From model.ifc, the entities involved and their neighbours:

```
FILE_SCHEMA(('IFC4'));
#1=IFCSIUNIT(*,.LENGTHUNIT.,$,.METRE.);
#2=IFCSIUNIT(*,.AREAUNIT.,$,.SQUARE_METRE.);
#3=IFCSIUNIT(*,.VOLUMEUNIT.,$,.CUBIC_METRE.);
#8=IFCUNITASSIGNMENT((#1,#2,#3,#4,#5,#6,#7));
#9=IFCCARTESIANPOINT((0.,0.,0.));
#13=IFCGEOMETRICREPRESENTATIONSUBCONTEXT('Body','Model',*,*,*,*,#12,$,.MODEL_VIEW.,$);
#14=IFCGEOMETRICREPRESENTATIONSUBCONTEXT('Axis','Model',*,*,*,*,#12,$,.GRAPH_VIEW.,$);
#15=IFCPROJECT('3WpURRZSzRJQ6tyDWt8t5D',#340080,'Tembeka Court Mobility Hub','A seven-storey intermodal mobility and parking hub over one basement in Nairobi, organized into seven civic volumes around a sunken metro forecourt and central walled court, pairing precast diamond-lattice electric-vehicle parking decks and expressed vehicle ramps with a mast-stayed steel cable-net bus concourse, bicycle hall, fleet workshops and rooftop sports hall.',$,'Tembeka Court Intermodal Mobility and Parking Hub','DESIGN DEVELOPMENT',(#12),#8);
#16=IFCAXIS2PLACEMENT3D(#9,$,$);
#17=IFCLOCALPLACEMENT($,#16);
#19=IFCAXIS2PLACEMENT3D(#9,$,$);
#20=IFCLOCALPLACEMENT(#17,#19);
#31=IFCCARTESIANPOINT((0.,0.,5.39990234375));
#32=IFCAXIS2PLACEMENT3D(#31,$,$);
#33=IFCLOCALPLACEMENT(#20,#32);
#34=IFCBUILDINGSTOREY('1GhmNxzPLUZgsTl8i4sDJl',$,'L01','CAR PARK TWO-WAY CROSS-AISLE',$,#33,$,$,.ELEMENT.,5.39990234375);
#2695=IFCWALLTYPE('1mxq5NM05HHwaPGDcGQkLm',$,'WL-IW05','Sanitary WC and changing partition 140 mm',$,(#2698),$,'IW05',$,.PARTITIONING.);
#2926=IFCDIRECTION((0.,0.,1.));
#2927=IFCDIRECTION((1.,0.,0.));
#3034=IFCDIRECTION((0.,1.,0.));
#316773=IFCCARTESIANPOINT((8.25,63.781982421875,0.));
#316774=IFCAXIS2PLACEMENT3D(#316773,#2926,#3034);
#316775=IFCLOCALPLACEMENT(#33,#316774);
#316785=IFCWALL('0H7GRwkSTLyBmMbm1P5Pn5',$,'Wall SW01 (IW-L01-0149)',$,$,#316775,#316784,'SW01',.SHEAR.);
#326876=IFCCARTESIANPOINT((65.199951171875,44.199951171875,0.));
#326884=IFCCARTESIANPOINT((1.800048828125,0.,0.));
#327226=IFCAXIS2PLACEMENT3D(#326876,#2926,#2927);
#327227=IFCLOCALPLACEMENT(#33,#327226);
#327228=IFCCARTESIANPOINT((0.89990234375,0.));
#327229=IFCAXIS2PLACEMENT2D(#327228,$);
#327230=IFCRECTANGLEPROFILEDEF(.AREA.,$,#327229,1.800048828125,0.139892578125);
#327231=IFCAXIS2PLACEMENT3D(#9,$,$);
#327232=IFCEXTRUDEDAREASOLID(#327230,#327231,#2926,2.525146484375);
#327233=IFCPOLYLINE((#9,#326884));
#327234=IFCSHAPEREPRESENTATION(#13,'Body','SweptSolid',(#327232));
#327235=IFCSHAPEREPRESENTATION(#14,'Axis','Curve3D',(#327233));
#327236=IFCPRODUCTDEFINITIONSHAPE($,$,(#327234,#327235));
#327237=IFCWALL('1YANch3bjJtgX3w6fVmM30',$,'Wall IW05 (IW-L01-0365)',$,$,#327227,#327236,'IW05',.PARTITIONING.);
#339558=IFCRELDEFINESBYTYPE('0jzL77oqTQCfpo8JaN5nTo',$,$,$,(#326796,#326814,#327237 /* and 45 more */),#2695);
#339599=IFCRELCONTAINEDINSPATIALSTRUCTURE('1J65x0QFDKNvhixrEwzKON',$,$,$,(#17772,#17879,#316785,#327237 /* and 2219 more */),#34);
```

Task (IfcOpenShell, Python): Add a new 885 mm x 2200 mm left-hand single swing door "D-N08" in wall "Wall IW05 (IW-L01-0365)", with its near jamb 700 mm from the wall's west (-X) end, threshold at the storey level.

```python
import numpy as np
import ifcopenshell
import ifcopenshell.api.feature
import ifcopenshell.api.geometry
import ifcopenshell.api.root
import ifcopenshell.api.spatial
import ifcopenshell.geom
import ifcopenshell.util.element
import ifcopenshell.util.placement
import ifcopenshell.util.representation
import ifcopenshell.util.shape
import ifcopenshell.util.unit

model = ifcopenshell.open("model.ifc")
unit_scale = ifcopenshell.util.unit.calculate_unit_scale(model)
settings = ifcopenshell.geom.settings()


def volume(element):
    """Net volume in cubic metres, openings subtracted."""
    shape = ifcopenshell.geom.create_shape(settings, element)
    return ifcopenshell.util.shape.get_volume(shape.geometry)


wall = model.by_id(327237)
storey = ifcopenshell.util.element.get_container(wall, ifc_class="IfcBuildingStorey")
context = ifcopenshell.util.representation.get_context(model, "Model", "Body", "MODEL_VIEW")
before = volume(wall)

width, height, from_end, sill = 0.885, 2.2, 0.7, 0.0  # metres

# The wall runs along its own X axis, and the end named is its -X end.
wall_shape = ifcopenshell.geom.create_shape(settings, wall)
x, y, z = ifcopenshell.util.shape.get_vertices(wall_shape.geometry).T
start = x.min() + from_end
face, thickness = float(y.min()), float(y.max() - y.min())
wall_matrix = ifcopenshell.util.placement.get_local_placement(wall.ObjectPlacement)
level = ifcopenshell.util.placement.get_local_placement(storey.ObjectPlacement)[2, 3]


def in_wall(x, y):
    """Placement at x, y metres in the wall's axes, at sill height."""
    matrix = wall_matrix.copy()
    matrix[:, 3] = wall_matrix @ np.array([x / unit_scale, y / unit_scale, 0.0, 1.0])
    matrix[2, 3] = level + sill / unit_scale
    return matrix


# Opening: a box that overshoots both wall faces by 50 mm.
opening = ifcopenshell.api.root.create_entity(model, ifc_class="IfcOpeningElement", predefined_type="OPENING")
box = ifcopenshell.api.geometry.add_wall_representation(
    model, context=context, length=width, height=height, thickness=thickness + 0.1
)
ifcopenshell.api.geometry.assign_representation(model, product=opening, representation=box)
ifcopenshell.api.geometry.edit_object_placement(model, product=opening, matrix=in_wall(start, face - 0.05), is_si=False)
ifcopenshell.api.feature.add_feature(model, feature=opening, element=wall)

door = ifcopenshell.api.root.create_entity(model, ifc_class="IfcDoor", name="D-N08", predefined_type="DOOR")
door.OverallWidth, door.OverallHeight = width / unit_scale, height / unit_scale
door.OperationType = "SINGLE_SWING_LEFT"
body = ifcopenshell.api.geometry.add_door_representation(
    model,
    context=context,
    overall_width=door.OverallWidth,
    overall_height=door.OverallHeight,
    operation_type="SINGLE_SWING_LEFT",
    lining_properties={"LiningDepth": thickness / unit_scale, "ThresholdDepth": thickness / unit_scale},
)
ifcopenshell.api.geometry.assign_representation(model, product=door, representation=body)
ifcopenshell.api.spatial.assign_container(model, products=[door], relating_structure=storey)
ifcopenshell.api.feature.add_filling(model, opening=opening, element=door)

# The lining spans the wall, so the door starts at the wall face.
ifcopenshell.api.geometry.edit_object_placement(model, product=door, matrix=in_wall(start, face), is_si=False)

after = volume(wall)

print(f"wall volume {before:.3f} -> {after:.3f} m3")

model.write("model_updated.ifc")
```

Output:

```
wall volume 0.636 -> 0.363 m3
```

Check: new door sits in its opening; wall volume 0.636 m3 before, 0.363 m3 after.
